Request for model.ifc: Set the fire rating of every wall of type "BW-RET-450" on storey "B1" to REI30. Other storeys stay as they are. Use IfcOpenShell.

First a look at what the model holds.

```python
import ifcopenshell
import ifcopenshell.util.element

model = ifcopenshell.open("model.ifc")
print(model.schema)
storey = next(s for s in model.by_type("IfcBuildingStorey") if s.Name == "B1")
walls = [e for e in ifcopenshell.util.element.get_decomposition(storey) if e.is_a("IfcWall")]
seen = {}
for e in walls:
    element_type = ifcopenshell.util.element.get_type(e)
    key = (element_type.Name if element_type != e and element_type else None, ifcopenshell.util.element.get_pset(e, "Pset_WallCommon", "FireRating"))
    seen[key] = seen.get(key, 0) + 1
for (name, value), count in sorted(seen.items(), key=str):
    print(count, "x", name, "|", value)
```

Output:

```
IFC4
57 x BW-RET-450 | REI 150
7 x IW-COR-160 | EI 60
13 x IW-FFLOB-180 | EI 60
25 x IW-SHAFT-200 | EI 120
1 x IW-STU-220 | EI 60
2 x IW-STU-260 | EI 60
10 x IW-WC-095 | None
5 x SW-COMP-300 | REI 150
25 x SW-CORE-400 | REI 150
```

```python
import ifcopenshell
import ifcopenshell.api.pset
import ifcopenshell.util.element

model = ifcopenshell.open("model.ifc")

storey = next(s for s in model.by_type("IfcBuildingStorey") if s.Name == "B1")
walls = [e for e in ifcopenshell.util.element.get_decomposition(storey) if e.is_a("IfcWall")]

count = 0
for e in walls:
    element_type = ifcopenshell.util.element.get_type(e)
    if element_type in (None, e) or element_type.Name != "BW-RET-450":
        continue
    # add_pset returns the element's existing set when there is one.
    pset = ifcopenshell.api.pset.add_pset(model, product=e, name="Pset_WallCommon")
    ifcopenshell.api.pset.edit_pset(model, pset=pset, properties={"FireRating": "REI30"})
    count += 1

print(count, "walls updated")

model.write("model_edited.ifc")
```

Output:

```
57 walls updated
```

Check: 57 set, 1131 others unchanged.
